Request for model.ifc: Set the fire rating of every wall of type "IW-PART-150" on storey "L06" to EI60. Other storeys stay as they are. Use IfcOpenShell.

First a look at what the model holds.

```python
import ifcopenshell
import ifcopenshell.util.element

model = ifcopenshell.open("model.ifc")
print(model.schema)
storey = next(s for s in model.by_type("IfcBuildingStorey") if s.Name == "L06")
walls = [e for e in ifcopenshell.util.element.get_decomposition(storey) if e.is_a("IfcWall")]
seen = {}
for e in walls:
    element_type = ifcopenshell.util.element.get_type(e)
    key = (element_type.Name if element_type != e and element_type else None, ifcopenshell.util.element.get_pset(e, "Pset_WallCommon", "FireRating"))
    seen[key] = seen.get(key, 0) + 1
for (name, value), count in sorted(seen.items(), key=str):
    print(count, "x", name, "|", value)
```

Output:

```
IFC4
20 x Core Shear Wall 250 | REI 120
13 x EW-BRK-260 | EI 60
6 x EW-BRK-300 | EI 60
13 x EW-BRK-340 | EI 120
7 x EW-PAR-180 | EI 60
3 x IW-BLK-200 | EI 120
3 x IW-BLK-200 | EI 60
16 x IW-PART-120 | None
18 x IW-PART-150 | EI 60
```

```python
import ifcopenshell
import ifcopenshell.api.pset
import ifcopenshell.util.element

model = ifcopenshell.open("model.ifc")

storey = next(s for s in model.by_type("IfcBuildingStorey") if s.Name == "L06")
walls = [e for e in ifcopenshell.util.element.get_decomposition(storey) if e.is_a("IfcWall")]

count = 0
for e in walls:
    element_type = ifcopenshell.util.element.get_type(e)
    if element_type in (None, e) or element_type.Name != "IW-PART-150":
        continue
    # add_pset returns the element's existing set when there is one.
    pset = ifcopenshell.api.pset.add_pset(model, product=e, name="Pset_WallCommon")
    ifcopenshell.api.pset.edit_pset(model, pset=pset, properties={"FireRating": "EI60"})
    count += 1

print(count, "walls updated")

model.write("model-out.ifc")
```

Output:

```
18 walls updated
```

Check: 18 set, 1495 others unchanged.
